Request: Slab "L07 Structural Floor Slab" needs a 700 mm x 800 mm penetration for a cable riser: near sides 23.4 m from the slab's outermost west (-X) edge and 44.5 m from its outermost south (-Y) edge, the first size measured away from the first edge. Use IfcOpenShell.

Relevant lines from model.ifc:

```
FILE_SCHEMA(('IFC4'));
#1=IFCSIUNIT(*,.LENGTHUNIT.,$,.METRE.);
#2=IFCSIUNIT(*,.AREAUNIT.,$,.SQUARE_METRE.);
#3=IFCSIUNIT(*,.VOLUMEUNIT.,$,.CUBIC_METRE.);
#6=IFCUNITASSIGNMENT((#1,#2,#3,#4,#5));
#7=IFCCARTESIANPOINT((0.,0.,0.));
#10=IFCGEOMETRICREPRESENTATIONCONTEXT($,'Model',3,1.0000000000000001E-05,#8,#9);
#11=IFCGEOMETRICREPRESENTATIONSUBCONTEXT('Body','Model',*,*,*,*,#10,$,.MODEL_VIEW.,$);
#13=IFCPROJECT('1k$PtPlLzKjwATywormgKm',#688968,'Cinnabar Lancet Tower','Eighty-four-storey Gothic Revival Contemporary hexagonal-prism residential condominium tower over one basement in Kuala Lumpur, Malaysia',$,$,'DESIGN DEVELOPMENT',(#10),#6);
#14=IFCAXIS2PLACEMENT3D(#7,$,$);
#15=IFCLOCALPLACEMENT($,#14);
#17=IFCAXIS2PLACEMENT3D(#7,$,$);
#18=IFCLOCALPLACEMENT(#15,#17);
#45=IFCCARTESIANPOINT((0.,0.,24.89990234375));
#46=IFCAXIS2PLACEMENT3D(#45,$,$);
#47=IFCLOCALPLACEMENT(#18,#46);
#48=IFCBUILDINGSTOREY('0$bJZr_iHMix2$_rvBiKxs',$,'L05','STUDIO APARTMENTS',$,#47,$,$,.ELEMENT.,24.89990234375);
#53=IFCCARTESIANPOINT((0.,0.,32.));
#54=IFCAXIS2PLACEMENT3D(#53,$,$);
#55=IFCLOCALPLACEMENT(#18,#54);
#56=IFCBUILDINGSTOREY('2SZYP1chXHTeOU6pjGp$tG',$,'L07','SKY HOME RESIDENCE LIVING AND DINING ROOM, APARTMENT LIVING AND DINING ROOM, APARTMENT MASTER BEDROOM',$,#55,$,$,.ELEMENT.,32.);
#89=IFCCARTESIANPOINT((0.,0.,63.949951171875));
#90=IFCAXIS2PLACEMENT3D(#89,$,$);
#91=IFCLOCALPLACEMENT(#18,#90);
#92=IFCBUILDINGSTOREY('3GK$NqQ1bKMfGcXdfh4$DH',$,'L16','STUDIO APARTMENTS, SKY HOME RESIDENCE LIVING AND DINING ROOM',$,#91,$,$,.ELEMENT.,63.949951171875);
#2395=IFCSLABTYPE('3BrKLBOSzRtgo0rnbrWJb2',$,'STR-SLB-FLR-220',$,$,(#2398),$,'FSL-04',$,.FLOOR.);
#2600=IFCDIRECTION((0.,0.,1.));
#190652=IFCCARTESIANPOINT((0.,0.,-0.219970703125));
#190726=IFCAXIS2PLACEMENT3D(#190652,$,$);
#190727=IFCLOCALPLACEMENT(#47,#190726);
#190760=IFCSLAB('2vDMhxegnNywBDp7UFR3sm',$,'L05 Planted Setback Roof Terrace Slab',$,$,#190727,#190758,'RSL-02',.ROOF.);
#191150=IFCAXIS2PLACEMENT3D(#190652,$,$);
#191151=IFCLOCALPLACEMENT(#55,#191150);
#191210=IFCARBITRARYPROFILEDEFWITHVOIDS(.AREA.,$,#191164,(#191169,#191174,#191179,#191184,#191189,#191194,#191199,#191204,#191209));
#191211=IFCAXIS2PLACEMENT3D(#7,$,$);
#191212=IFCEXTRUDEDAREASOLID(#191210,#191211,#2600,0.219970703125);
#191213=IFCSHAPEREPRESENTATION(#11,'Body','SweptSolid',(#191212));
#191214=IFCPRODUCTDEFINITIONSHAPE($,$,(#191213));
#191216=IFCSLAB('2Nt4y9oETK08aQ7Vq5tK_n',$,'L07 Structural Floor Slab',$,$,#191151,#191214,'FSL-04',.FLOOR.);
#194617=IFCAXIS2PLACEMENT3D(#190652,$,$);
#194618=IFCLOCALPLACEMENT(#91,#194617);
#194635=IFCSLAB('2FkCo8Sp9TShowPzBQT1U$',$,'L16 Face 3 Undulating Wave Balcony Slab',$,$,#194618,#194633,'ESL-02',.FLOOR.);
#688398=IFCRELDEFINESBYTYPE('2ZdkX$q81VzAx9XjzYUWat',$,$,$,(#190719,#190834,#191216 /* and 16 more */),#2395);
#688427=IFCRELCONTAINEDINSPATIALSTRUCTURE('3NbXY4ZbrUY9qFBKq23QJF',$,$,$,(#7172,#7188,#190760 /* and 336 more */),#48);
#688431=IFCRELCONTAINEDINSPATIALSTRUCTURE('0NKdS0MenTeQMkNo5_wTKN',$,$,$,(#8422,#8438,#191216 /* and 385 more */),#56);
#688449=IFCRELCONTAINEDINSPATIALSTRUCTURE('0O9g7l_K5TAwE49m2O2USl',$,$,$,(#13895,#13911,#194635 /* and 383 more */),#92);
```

```python
import numpy as np
import ifcopenshell
import ifcopenshell.api.feature
import ifcopenshell.api.geometry
import ifcopenshell.api.root
import ifcopenshell.geom
import ifcopenshell.util.placement
import ifcopenshell.util.representation
import ifcopenshell.util.shape
import ifcopenshell.util.unit

model = ifcopenshell.open("model.ifc")
unit_scale = ifcopenshell.util.unit.calculate_unit_scale(model)
settings = ifcopenshell.geom.settings()


def volume(element):
    """Net volume in cubic metres, openings subtracted."""
    shape = ifcopenshell.geom.create_shape(settings, element)
    return ifcopenshell.util.shape.get_volume(shape.geometry)


slab = model.by_guid("2Nt4y9oETK08aQ7Vq5tK_n")
before = volume(slab)

# Extent in the slab's own axes, in metres. The edges named are its -X and -Y sides.
slab_shape = ifcopenshell.geom.create_shape(settings, slab)
vertices = ifcopenshell.util.shape.get_vertices(slab_shape.geometry)
x_min, y_min, bottom = vertices.min(axis=0)
top = vertices[:, 2].max()

opening = ifcopenshell.api.root.create_entity(model, ifc_class="IfcOpeningElement", name="Cable riser opening", predefined_type="OPENING")
context = ifcopenshell.util.representation.get_context(model, "Model", "Body", "MODEL_VIEW")
width, depth = 0.7, 0.8
outline = [(0.0, 0.0), (width, 0.0), (width, depth), (0.0, depth), (0.0, 0.0)]
# Overshoot both faces by 50 mm so the cut is clean.
shape = ifcopenshell.api.geometry.add_slab_representation(
    model, context=context, depth=top - bottom + 0.1, polyline=outline
)
ifcopenshell.api.geometry.assign_representation(model, product=opening, representation=shape)

matrix = ifcopenshell.util.placement.get_local_placement(slab.ObjectPlacement)
matrix[:, 3] = matrix @ np.append(np.array([x_min + 23.4, y_min + 44.5, bottom - 0.05]) / unit_scale, 1.0)
ifcopenshell.api.geometry.edit_object_placement(model, product=opening, matrix=matrix, is_si=False)
ifcopenshell.api.feature.add_feature(model, feature=opening, element=slab)

after = volume(slab)

print(f"slab volume {before:.3f} -> {after:.3f} m3")

model.write("model_rev.ifc")
```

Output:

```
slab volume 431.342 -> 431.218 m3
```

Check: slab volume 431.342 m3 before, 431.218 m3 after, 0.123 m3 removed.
